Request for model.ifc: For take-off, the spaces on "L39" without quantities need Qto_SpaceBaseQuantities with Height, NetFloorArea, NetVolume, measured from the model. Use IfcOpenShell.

First a look at what the model holds.

```python
import ifcopenshell
import ifcopenshell.util.element
import ifcopenshell.util.unit

model = ifcopenshell.open("model.ifc")
print(model.schema)
for unit_type in ("LENGTHUNIT", "AREAUNIT", "VOLUMEUNIT"):
    print(unit_type, ifcopenshell.util.unit.calculate_unit_scale(model, unit_type))
storey = next(s for s in model.by_type("IfcBuildingStorey") if s.Name == "L39")
spaces = [e for e in ifcopenshell.util.element.get_decomposition(storey) if e.is_a("IfcSpace")]
for e in sorted(spaces, key=lambda e: e.id()):
    print(e.id(), e.is_a(), e.Name, list(ifcopenshell.util.element.get_psets(e, qtos_only=True)), sep=" | ")
```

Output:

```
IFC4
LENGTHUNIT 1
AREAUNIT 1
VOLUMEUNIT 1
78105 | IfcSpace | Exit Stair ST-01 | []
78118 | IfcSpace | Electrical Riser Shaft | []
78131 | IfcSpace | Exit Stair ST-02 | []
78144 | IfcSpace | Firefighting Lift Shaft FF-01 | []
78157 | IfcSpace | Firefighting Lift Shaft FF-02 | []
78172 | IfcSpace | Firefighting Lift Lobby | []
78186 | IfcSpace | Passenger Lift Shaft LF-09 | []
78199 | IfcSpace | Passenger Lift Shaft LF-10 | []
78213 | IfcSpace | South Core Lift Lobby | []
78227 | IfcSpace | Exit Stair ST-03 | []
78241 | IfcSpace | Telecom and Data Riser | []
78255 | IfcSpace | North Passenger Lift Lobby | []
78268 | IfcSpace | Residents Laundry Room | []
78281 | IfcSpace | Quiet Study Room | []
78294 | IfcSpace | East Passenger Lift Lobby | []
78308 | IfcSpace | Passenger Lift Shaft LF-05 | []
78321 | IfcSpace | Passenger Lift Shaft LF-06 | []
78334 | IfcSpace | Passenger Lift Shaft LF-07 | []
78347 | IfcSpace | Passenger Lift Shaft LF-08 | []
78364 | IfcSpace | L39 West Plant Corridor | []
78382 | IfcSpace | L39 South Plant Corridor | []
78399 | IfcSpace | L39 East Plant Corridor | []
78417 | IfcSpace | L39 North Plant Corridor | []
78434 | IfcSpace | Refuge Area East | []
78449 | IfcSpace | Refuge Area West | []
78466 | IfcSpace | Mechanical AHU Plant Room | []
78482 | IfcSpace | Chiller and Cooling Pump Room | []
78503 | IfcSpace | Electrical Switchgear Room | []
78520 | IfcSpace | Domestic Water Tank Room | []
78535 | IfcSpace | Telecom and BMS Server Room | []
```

```python
import ifcopenshell
import ifcopenshell.api.pset
import ifcopenshell.geom
import ifcopenshell.util.element
import ifcopenshell.util.shape
import ifcopenshell.util.unit

model = ifcopenshell.open("model.ifc")
unit_scale = ifcopenshell.util.unit.calculate_unit_scale(model)
area_scale = ifcopenshell.util.unit.calculate_unit_scale(model, "AREAUNIT")
volume_scale = ifcopenshell.util.unit.calculate_unit_scale(model, "VOLUMEUNIT")
settings = ifcopenshell.geom.settings()

storey = next(s for s in model.by_type("IfcBuildingStorey") if s.Name == "L39")
spaces = [e for e in ifcopenshell.util.element.get_decomposition(storey) if e.is_a("IfcSpace")]

for e in sorted(spaces, key=lambda e: e.id()):
    if ifcopenshell.util.element.get_psets(e, qtos_only=True, should_inherit=False):
        continue
    # Geometry comes back in metres, in the element's own axes.
    shape = ifcopenshell.geom.create_shape(settings, e)
    values = {
        "Height": ifcopenshell.util.shape.get_z(shape.geometry) / unit_scale,
        "NetFloorArea": ifcopenshell.util.shape.get_footprint_area(shape.geometry) / area_scale,
        "NetVolume": ifcopenshell.util.shape.get_volume(shape.geometry) / volume_scale,
    }
    qto = ifcopenshell.api.pset.add_qto(model, product=e, name="Qto_SpaceBaseQuantities")
    ifcopenshell.api.pset.edit_qto(model, qto=qto, properties=values)
    print(e.id(), {k: round(v, 3) for k, v in values.items()})

model.write("model_edited.ifc")
```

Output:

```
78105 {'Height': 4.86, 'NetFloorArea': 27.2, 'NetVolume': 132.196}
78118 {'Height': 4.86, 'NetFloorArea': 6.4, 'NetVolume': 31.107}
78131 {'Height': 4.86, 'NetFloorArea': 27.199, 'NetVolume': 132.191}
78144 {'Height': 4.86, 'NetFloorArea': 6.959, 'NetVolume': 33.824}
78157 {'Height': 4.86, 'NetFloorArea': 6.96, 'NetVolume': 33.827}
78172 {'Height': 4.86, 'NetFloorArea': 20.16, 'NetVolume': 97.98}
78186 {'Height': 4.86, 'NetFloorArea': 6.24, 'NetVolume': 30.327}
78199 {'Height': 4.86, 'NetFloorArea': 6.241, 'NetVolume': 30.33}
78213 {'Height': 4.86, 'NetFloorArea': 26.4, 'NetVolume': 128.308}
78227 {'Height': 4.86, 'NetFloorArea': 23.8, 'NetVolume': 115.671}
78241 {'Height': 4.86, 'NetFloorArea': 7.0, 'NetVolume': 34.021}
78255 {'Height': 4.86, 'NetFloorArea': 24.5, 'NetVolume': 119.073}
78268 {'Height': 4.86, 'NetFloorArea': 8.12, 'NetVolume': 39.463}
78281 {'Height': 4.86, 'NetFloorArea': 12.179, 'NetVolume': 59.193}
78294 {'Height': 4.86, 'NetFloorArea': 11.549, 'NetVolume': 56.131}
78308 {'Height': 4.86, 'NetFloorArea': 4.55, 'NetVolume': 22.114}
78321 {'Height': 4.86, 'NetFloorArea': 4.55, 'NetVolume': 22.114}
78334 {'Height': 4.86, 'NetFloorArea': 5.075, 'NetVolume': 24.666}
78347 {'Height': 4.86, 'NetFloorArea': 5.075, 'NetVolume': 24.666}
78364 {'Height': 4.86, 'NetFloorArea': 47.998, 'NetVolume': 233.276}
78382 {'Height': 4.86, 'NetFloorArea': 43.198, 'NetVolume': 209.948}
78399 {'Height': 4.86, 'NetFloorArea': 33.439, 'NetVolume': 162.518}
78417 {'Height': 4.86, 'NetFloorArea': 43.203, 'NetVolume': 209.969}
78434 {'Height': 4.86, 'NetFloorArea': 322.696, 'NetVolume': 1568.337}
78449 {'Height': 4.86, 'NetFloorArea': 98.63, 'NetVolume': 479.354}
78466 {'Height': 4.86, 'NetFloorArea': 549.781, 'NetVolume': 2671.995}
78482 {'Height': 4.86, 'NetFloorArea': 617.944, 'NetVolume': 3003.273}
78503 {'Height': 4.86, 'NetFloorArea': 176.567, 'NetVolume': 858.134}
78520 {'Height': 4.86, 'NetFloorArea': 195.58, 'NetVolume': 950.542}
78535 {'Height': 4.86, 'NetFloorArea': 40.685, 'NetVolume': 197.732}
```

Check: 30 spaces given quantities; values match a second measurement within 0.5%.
